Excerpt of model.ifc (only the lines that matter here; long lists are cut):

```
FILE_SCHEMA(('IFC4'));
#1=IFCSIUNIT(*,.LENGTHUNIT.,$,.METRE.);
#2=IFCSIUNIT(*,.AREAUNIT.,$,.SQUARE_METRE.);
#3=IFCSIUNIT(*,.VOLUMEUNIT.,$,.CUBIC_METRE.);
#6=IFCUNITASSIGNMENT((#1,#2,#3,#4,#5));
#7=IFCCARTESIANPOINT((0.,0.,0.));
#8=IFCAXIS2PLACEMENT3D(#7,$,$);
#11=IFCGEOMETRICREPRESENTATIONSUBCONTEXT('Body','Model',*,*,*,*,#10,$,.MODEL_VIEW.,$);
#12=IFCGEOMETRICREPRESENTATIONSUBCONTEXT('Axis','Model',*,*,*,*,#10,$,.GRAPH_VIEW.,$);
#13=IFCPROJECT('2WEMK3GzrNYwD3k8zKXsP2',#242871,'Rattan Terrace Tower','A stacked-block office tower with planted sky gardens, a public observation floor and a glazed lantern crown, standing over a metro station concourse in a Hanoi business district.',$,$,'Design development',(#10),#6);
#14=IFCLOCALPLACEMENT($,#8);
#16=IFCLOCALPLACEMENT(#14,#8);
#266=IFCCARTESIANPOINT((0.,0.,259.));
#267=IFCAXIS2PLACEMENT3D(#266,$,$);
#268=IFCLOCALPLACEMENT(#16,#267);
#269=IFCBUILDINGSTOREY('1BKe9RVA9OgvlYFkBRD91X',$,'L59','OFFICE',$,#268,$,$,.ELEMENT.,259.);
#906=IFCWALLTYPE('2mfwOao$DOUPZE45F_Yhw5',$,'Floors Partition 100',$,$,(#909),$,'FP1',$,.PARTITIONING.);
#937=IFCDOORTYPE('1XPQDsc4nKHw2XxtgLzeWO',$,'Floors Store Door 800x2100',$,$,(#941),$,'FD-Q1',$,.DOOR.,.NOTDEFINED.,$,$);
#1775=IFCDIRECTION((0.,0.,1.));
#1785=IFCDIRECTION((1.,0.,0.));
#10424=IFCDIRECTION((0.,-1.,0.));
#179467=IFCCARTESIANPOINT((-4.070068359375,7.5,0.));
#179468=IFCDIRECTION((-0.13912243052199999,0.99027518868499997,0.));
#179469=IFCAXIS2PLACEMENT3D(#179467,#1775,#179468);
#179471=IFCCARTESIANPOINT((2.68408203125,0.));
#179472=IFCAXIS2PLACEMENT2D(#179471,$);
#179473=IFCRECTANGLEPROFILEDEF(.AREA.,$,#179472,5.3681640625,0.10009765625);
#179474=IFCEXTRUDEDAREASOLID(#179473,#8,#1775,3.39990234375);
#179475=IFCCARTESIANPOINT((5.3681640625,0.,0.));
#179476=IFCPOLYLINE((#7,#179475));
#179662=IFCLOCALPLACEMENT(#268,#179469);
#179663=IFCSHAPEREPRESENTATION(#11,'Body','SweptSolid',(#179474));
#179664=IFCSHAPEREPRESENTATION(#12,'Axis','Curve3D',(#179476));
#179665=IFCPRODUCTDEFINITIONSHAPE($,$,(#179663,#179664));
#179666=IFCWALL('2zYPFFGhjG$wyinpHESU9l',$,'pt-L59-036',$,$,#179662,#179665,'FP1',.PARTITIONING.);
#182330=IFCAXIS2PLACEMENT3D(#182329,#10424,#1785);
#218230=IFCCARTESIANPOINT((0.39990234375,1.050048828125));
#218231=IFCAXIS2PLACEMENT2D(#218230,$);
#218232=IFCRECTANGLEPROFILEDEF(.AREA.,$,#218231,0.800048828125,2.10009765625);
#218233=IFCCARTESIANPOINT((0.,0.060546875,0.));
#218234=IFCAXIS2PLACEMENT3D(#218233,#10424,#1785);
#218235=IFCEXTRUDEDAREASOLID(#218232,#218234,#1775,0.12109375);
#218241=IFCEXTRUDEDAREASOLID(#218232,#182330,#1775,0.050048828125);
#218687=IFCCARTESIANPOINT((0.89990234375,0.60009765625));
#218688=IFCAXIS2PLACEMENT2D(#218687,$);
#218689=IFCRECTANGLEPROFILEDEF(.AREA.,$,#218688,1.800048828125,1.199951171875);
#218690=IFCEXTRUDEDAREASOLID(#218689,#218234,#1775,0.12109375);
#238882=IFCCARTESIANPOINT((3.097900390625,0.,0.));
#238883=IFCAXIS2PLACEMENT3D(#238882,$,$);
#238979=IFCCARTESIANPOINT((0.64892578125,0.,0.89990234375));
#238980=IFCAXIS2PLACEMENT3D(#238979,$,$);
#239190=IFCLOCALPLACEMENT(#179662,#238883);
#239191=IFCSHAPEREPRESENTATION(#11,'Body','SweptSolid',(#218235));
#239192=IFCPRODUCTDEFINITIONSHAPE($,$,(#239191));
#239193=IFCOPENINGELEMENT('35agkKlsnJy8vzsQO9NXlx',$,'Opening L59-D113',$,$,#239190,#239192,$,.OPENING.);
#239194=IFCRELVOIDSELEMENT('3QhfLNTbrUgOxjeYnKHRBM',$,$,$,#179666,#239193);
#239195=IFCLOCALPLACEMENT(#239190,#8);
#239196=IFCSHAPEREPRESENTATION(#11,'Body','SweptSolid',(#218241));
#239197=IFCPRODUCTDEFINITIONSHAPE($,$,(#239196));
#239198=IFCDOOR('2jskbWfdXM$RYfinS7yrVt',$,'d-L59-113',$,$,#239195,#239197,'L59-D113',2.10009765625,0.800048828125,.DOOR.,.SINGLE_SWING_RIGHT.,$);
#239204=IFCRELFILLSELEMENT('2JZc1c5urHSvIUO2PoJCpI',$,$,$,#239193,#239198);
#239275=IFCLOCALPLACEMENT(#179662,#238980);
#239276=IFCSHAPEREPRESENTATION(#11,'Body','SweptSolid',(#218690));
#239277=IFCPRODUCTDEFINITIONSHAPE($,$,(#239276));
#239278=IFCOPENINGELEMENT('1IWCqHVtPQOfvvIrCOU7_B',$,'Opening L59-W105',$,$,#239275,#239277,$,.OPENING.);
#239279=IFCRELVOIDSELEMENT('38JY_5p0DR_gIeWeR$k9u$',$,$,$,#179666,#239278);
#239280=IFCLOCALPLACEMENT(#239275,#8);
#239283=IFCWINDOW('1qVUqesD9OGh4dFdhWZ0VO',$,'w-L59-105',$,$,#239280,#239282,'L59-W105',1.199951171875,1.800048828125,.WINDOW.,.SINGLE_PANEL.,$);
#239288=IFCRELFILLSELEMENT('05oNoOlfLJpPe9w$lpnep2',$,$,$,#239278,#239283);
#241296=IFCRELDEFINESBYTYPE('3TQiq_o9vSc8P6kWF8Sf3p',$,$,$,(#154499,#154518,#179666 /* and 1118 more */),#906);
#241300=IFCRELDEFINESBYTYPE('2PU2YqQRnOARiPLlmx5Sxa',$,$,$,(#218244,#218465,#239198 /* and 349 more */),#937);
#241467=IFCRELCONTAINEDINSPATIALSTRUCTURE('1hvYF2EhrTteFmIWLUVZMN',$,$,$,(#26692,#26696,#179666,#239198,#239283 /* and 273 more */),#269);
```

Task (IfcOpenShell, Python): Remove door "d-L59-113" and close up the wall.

```python
import ifcopenshell
import ifcopenshell.api.feature
import ifcopenshell.api.root
import ifcopenshell.geom
import ifcopenshell.util.shape

model = ifcopenshell.open("model.ifc")
settings = ifcopenshell.geom.settings()


def volume(element):
    """Net volume in cubic metres, openings subtracted."""
    shape = ifcopenshell.geom.create_shape(settings, element)
    return ifcopenshell.util.shape.get_volume(shape.geometry)


door = model.by_guid("2jskbWfdXM$RYfinS7yrVt")
opening = door.FillsVoids[0].RelatingOpeningElement
wall = opening.VoidsElements[0].RelatingBuildingElement
before = volume(wall)

ifcopenshell.api.root.remove_product(model, product=door)
ifcopenshell.api.feature.remove_feature(model, feature=opening)

after = volume(wall)

print(f"wall volume {before:.3f} -> {after:.3f} m3")

model.write("model_rev.ifc")
```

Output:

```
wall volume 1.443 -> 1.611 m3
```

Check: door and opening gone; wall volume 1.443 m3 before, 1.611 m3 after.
